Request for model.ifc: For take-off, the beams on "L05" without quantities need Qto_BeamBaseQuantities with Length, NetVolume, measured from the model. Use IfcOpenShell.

First a look at what the model holds.

```python
import ifcopenshell
import ifcopenshell.util.element
import ifcopenshell.util.unit

model = ifcopenshell.open("model.ifc")
print(model.schema)
for unit_type in ("LENGTHUNIT", "AREAUNIT", "VOLUMEUNIT"):
    print(unit_type, ifcopenshell.util.unit.calculate_unit_scale(model, unit_type))
storey = next(s for s in model.by_type("IfcBuildingStorey") if s.Name == "L05")
beams = [e for e in ifcopenshell.util.element.get_decomposition(storey) if e.is_a("IfcBeam")]
for e in sorted(beams, key=lambda e: e.id()):
    print(e.id(), e.is_a(), e.Name, list(ifcopenshell.util.element.get_psets(e, qtos_only=True)), sep=" | ")
```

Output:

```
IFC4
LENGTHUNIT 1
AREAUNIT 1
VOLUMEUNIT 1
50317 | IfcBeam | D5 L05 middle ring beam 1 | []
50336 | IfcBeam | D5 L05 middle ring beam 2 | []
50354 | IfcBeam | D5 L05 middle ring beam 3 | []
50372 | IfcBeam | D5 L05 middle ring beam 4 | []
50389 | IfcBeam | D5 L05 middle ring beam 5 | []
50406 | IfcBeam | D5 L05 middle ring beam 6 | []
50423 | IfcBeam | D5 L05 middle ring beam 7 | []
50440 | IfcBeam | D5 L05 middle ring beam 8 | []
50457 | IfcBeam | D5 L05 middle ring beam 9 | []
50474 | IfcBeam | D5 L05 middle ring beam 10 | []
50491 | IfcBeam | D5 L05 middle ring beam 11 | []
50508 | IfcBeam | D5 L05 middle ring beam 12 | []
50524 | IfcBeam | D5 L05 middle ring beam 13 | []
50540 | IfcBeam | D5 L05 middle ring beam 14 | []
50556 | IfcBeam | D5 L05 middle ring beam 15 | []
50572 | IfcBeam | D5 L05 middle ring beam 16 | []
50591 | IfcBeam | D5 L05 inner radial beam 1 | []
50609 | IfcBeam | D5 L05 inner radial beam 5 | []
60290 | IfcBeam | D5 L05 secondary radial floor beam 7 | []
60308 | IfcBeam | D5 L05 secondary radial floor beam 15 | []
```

```python
import ifcopenshell
import ifcopenshell.api.pset
import ifcopenshell.geom
import ifcopenshell.util.element
import ifcopenshell.util.shape
import ifcopenshell.util.unit

model = ifcopenshell.open("model.ifc")
unit_scale = ifcopenshell.util.unit.calculate_unit_scale(model)
volume_scale = ifcopenshell.util.unit.calculate_unit_scale(model, "VOLUMEUNIT")
settings = ifcopenshell.geom.settings()

storey = next(s for s in model.by_type("IfcBuildingStorey") if s.Name == "L05")
beams = [e for e in ifcopenshell.util.element.get_decomposition(storey) if e.is_a("IfcBeam")]

for e in sorted(beams, key=lambda e: e.id()):
    if ifcopenshell.util.element.get_psets(e, qtos_only=True, should_inherit=False):
        continue
    # Geometry comes back in metres, in the element's own axes.
    shape = ifcopenshell.geom.create_shape(settings, e)
    values = {
        "Length": ifcopenshell.util.shape.get_max_xyz(shape.geometry) / unit_scale,
        "NetVolume": ifcopenshell.util.shape.get_volume(shape.geometry) / volume_scale,
    }
    qto = ifcopenshell.api.pset.add_qto(model, product=e, name="Qto_BeamBaseQuantities")
    ifcopenshell.api.pset.edit_qto(model, qto=qto, properties=values)
    print(e.id(), {k: round(v, 3) for k, v in values.items()})

model.write("model_v2.ifc")
```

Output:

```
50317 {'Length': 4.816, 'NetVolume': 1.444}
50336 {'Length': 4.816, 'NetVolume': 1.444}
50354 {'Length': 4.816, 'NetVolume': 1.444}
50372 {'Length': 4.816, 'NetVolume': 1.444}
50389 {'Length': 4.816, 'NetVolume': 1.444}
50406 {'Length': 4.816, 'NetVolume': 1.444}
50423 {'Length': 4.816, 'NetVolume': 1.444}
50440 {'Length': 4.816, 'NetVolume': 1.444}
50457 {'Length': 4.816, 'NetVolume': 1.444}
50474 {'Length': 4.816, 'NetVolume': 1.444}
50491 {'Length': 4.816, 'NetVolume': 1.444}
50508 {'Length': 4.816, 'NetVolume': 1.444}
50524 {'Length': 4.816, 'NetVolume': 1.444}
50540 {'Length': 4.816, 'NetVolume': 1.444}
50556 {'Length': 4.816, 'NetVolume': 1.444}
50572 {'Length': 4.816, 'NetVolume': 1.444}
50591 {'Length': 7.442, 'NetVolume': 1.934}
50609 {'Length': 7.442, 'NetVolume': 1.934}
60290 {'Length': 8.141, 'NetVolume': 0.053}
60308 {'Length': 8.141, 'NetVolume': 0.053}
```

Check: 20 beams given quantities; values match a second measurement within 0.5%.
